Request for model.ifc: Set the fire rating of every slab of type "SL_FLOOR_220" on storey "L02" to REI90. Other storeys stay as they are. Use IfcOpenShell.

First a look at what the model holds.

```python
import ifcopenshell
import ifcopenshell.util.element

model = ifcopenshell.open("model.ifc")
print(model.schema)
storey = next(s for s in model.by_type("IfcBuildingStorey") if s.Name == "L02")
slabs = [e for e in ifcopenshell.util.element.get_decomposition(storey) if e.is_a("IfcSlab")]
seen = {}
for e in slabs:
    element_type = ifcopenshell.util.element.get_type(e)
    key = (element_type.Name if element_type != e and element_type else None, ifcopenshell.util.element.get_pset(e, "Pset_SlabCommon", "FireRating"))
    seen[key] = seen.get(key, 0) + 1
for (name, value), count in sorted(seen.items(), key=str):
    print(count, "x", name, "|", value)
```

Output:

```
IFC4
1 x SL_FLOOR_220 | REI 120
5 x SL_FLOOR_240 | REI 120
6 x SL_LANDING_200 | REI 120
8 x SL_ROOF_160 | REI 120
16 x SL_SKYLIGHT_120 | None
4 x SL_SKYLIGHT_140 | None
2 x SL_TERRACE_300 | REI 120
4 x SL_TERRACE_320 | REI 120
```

```python
import ifcopenshell
import ifcopenshell.api.pset
import ifcopenshell.util.element

model = ifcopenshell.open("model.ifc")

storey = next(s for s in model.by_type("IfcBuildingStorey") if s.Name == "L02")
slabs = [e for e in ifcopenshell.util.element.get_decomposition(storey) if e.is_a("IfcSlab")]

count = 0
for e in slabs:
    element_type = ifcopenshell.util.element.get_type(e)
    if element_type in (None, e) or element_type.Name != "SL_FLOOR_220":
        continue
    # add_pset returns the element's existing set when there is one.
    pset = ifcopenshell.api.pset.add_pset(model, product=e, name="Pset_SlabCommon")
    ifcopenshell.api.pset.edit_pset(model, pset=pset, properties={"FireRating": "REI90"})
    count += 1

print(count, "slabs updated")

model.write("model_v2.ifc")
```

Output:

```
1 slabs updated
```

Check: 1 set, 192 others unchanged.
